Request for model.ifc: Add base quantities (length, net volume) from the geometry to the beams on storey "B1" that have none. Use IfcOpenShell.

First a look at what the model holds.

```python
import ifcopenshell
import ifcopenshell.util.element
import ifcopenshell.util.unit

model = ifcopenshell.open("model.ifc")
print(model.schema)
for unit_type in ("LENGTHUNIT", "AREAUNIT", "VOLUMEUNIT"):
    print(unit_type, ifcopenshell.util.unit.calculate_unit_scale(model, unit_type))
storey = next(s for s in model.by_type("IfcBuildingStorey") if s.Name == "B1")
beams = [e for e in ifcopenshell.util.element.get_decomposition(storey) if e.is_a("IfcBeam")]
for e in sorted(beams, key=lambda e: e.id()):
    print(e.id(), e.is_a(), e.Name, list(ifcopenshell.util.element.get_psets(e, qtos_only=True)), sep=" | ")
```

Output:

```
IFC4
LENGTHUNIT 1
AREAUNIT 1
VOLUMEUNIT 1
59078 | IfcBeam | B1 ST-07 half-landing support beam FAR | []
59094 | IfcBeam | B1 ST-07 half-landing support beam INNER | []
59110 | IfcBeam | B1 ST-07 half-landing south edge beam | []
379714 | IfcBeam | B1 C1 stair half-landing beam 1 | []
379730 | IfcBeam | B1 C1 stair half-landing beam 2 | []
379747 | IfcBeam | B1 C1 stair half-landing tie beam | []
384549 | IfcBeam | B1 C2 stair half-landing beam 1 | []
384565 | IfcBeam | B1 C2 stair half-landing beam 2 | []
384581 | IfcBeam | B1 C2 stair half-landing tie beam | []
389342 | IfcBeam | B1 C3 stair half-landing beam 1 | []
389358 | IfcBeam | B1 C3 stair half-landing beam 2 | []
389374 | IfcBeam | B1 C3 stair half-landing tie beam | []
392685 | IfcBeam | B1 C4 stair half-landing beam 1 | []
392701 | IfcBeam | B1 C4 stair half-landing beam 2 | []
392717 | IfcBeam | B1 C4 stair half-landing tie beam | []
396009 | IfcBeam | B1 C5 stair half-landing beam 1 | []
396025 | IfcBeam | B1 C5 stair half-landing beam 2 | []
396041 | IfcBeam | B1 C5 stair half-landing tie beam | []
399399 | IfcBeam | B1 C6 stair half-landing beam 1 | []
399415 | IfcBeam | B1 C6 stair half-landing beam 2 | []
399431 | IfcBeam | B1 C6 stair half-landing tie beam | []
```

```python
import ifcopenshell
import ifcopenshell.api.pset
import ifcopenshell.geom
import ifcopenshell.util.element
import ifcopenshell.util.shape
import ifcopenshell.util.unit

model = ifcopenshell.open("model.ifc")
unit_scale = ifcopenshell.util.unit.calculate_unit_scale(model)
volume_scale = ifcopenshell.util.unit.calculate_unit_scale(model, "VOLUMEUNIT")
settings = ifcopenshell.geom.settings()

storey = next(s for s in model.by_type("IfcBuildingStorey") if s.Name == "B1")
beams = [e for e in ifcopenshell.util.element.get_decomposition(storey) if e.is_a("IfcBeam")]

for e in sorted(beams, key=lambda e: e.id()):
    if ifcopenshell.util.element.get_psets(e, qtos_only=True, should_inherit=False):
        continue
    # Geometry comes back in metres, in the element's own axes.
    shape = ifcopenshell.geom.create_shape(settings, e)
    values = {
        "Length": ifcopenshell.util.shape.get_max_xyz(shape.geometry) / unit_scale,
        "NetVolume": ifcopenshell.util.shape.get_volume(shape.geometry) / volume_scale,
    }
    qto = ifcopenshell.api.pset.add_qto(model, product=e, name="Qto_BeamBaseQuantities")
    ifcopenshell.api.pset.edit_qto(model, qto=qto, properties=values)
    print(e.id(), {k: round(v, 3) for k, v in values.items()})

model.write("model_v2.ifc")
```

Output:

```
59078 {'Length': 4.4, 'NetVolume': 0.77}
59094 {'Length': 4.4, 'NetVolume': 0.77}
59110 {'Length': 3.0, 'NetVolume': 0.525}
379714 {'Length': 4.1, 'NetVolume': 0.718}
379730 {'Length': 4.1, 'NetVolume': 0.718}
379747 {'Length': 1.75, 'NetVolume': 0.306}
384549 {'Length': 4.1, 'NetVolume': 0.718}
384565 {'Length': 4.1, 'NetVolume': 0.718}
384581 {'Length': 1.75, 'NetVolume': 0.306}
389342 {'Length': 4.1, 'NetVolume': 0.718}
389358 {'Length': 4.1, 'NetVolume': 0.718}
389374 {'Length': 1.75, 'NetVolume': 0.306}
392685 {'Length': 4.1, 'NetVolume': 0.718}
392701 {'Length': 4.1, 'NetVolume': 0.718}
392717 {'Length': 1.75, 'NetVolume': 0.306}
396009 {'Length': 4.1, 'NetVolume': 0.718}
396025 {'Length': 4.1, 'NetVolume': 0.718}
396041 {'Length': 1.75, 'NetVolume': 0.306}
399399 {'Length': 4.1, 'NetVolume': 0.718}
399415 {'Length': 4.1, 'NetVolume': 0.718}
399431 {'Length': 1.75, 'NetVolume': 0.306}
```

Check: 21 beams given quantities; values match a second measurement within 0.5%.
